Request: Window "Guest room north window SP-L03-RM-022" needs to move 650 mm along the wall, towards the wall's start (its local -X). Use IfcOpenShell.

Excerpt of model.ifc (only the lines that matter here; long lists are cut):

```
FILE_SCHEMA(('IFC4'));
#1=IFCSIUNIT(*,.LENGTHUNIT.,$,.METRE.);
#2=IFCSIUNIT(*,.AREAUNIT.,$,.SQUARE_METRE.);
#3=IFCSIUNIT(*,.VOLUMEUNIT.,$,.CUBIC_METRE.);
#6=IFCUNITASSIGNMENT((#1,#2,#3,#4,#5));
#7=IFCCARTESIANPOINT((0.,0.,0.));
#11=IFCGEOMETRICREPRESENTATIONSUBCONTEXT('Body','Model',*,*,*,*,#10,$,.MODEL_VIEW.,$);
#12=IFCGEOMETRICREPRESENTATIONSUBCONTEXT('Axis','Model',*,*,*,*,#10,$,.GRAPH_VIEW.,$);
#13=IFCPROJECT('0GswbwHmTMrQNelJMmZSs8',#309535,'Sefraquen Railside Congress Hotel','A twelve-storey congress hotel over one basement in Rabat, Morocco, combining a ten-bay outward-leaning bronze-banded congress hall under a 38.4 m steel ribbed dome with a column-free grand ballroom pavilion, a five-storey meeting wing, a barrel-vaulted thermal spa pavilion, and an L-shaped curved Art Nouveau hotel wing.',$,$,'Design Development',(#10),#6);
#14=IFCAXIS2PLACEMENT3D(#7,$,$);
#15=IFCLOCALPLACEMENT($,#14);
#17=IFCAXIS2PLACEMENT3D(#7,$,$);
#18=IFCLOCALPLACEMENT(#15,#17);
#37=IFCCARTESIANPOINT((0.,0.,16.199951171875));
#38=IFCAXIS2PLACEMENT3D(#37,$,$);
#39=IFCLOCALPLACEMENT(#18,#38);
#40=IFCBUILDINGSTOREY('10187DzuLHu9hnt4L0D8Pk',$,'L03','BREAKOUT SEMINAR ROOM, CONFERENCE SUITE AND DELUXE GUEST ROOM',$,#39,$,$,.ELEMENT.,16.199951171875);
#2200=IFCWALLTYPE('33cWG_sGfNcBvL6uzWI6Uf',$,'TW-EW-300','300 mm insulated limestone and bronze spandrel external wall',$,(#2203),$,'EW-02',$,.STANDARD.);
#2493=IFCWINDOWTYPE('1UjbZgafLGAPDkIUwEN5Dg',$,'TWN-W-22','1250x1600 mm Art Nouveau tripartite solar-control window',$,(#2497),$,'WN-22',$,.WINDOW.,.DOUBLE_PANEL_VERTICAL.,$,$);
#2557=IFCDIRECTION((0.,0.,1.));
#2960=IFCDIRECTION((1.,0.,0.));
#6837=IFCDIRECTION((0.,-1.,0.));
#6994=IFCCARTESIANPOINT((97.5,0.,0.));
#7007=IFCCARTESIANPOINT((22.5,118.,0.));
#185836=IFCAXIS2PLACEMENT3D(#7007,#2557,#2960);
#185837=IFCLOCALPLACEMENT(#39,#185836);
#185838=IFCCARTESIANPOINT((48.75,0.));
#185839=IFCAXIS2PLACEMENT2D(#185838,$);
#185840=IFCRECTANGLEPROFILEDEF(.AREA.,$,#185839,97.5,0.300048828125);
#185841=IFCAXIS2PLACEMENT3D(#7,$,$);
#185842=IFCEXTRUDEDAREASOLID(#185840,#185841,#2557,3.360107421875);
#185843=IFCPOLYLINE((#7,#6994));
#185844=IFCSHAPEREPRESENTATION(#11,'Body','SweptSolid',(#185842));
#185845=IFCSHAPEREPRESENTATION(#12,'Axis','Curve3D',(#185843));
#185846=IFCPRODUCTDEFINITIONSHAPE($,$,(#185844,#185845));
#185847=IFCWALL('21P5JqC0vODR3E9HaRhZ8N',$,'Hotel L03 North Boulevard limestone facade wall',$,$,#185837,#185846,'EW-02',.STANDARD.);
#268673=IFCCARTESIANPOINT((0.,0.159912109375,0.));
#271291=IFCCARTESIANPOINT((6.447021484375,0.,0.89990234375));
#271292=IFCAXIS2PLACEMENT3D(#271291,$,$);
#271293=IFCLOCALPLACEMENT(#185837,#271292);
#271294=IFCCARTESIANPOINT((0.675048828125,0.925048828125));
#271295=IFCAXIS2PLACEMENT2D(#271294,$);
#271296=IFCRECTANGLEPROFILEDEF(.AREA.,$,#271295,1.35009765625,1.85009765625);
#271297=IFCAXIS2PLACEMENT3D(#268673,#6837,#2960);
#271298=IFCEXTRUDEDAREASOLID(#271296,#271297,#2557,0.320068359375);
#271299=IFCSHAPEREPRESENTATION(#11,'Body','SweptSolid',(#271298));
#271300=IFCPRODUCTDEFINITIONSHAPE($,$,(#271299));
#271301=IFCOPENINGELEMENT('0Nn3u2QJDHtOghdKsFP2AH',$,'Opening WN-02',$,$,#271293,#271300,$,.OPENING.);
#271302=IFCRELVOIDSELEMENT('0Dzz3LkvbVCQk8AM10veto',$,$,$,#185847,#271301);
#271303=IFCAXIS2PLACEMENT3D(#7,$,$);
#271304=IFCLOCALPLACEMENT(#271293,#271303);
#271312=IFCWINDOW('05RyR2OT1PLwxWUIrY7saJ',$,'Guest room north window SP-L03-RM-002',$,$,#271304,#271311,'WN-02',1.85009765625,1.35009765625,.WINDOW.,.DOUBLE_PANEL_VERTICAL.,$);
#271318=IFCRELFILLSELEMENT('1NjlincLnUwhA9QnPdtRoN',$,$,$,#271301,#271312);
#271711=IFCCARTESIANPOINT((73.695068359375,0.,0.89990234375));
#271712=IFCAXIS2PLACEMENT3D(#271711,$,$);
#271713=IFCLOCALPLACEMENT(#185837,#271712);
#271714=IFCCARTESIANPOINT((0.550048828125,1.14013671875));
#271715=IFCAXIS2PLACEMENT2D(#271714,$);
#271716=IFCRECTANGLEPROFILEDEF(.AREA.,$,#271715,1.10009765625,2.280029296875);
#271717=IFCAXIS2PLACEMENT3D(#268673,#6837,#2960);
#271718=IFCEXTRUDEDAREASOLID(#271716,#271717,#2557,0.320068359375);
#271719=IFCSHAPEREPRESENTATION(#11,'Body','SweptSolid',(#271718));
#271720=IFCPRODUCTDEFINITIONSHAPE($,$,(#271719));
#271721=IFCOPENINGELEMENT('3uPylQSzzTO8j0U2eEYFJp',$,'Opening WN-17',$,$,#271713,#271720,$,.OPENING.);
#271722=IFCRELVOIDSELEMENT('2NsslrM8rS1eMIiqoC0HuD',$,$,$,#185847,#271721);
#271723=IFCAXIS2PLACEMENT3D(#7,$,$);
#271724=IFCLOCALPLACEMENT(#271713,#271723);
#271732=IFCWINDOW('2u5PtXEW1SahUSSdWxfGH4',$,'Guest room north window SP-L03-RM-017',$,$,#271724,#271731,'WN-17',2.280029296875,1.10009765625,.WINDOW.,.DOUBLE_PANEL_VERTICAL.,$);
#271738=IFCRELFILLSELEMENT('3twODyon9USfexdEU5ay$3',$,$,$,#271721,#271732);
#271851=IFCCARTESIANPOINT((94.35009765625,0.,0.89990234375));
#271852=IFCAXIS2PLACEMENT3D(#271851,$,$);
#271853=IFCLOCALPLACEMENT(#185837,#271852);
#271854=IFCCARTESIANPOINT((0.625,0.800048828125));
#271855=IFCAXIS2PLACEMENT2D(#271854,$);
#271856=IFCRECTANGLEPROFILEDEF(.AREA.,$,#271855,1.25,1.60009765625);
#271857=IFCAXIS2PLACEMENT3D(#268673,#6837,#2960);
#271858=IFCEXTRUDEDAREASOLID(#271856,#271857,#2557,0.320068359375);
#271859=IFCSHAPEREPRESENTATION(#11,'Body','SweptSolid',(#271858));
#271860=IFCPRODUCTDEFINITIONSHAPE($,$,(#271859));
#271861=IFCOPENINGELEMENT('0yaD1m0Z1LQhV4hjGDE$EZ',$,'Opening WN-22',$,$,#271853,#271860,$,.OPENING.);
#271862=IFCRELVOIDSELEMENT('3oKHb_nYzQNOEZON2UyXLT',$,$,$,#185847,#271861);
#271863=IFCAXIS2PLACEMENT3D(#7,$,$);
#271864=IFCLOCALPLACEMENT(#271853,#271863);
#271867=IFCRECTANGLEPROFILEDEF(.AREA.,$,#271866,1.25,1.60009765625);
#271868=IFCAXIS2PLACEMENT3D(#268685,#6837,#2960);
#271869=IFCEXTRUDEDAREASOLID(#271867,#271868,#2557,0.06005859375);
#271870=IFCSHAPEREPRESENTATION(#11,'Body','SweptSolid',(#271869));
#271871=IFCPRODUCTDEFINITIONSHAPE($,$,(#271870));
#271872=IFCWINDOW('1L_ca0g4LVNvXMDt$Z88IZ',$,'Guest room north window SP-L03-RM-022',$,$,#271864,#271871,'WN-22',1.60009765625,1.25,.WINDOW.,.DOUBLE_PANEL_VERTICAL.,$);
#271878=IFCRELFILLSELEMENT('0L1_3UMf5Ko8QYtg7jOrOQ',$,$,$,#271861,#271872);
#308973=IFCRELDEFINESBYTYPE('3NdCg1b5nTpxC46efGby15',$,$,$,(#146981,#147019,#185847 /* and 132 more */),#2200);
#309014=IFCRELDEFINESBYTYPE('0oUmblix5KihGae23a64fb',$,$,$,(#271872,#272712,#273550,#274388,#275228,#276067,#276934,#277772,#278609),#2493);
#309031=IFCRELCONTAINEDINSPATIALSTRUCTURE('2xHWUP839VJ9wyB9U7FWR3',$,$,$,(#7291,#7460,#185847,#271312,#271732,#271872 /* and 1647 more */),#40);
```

```python
import ifcopenshell
import ifcopenshell.api.geometry
import ifcopenshell.util.placement
import ifcopenshell.util.unit

model = ifcopenshell.open("model.ifc")
unit_scale = ifcopenshell.util.unit.calculate_unit_scale(model)

window = model.by_guid("1L_ca0g4LVNvXMDt$Z88IZ")
opening = window.FillsVoids[0].RelatingOpeningElement
wall = opening.VoidsElements[0].RelatingBuildingElement

wall_matrix = ifcopenshell.util.placement.get_local_placement(wall.ObjectPlacement)
shift = wall_matrix[:3, 0] * -0.65 / unit_scale
before = ifcopenshell.util.placement.get_local_placement(window.ObjectPlacement)[:3, 3].copy()

# The window is placed relative to its opening, so it follows when the opening moves.
matrix = ifcopenshell.util.placement.get_local_placement(opening.ObjectPlacement)
matrix[:3, 3] += shift
ifcopenshell.api.geometry.edit_object_placement(
    model, product=opening, matrix=matrix, is_si=False, should_transform_children=True
)

after = ifcopenshell.util.placement.get_local_placement(window.ObjectPlacement)[:3, 3]
print("window moved by", (after - before).round(3) + 0.0)

model.write("model-out.ifc")
```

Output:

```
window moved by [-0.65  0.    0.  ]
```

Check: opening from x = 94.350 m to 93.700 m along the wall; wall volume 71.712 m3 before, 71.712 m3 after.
